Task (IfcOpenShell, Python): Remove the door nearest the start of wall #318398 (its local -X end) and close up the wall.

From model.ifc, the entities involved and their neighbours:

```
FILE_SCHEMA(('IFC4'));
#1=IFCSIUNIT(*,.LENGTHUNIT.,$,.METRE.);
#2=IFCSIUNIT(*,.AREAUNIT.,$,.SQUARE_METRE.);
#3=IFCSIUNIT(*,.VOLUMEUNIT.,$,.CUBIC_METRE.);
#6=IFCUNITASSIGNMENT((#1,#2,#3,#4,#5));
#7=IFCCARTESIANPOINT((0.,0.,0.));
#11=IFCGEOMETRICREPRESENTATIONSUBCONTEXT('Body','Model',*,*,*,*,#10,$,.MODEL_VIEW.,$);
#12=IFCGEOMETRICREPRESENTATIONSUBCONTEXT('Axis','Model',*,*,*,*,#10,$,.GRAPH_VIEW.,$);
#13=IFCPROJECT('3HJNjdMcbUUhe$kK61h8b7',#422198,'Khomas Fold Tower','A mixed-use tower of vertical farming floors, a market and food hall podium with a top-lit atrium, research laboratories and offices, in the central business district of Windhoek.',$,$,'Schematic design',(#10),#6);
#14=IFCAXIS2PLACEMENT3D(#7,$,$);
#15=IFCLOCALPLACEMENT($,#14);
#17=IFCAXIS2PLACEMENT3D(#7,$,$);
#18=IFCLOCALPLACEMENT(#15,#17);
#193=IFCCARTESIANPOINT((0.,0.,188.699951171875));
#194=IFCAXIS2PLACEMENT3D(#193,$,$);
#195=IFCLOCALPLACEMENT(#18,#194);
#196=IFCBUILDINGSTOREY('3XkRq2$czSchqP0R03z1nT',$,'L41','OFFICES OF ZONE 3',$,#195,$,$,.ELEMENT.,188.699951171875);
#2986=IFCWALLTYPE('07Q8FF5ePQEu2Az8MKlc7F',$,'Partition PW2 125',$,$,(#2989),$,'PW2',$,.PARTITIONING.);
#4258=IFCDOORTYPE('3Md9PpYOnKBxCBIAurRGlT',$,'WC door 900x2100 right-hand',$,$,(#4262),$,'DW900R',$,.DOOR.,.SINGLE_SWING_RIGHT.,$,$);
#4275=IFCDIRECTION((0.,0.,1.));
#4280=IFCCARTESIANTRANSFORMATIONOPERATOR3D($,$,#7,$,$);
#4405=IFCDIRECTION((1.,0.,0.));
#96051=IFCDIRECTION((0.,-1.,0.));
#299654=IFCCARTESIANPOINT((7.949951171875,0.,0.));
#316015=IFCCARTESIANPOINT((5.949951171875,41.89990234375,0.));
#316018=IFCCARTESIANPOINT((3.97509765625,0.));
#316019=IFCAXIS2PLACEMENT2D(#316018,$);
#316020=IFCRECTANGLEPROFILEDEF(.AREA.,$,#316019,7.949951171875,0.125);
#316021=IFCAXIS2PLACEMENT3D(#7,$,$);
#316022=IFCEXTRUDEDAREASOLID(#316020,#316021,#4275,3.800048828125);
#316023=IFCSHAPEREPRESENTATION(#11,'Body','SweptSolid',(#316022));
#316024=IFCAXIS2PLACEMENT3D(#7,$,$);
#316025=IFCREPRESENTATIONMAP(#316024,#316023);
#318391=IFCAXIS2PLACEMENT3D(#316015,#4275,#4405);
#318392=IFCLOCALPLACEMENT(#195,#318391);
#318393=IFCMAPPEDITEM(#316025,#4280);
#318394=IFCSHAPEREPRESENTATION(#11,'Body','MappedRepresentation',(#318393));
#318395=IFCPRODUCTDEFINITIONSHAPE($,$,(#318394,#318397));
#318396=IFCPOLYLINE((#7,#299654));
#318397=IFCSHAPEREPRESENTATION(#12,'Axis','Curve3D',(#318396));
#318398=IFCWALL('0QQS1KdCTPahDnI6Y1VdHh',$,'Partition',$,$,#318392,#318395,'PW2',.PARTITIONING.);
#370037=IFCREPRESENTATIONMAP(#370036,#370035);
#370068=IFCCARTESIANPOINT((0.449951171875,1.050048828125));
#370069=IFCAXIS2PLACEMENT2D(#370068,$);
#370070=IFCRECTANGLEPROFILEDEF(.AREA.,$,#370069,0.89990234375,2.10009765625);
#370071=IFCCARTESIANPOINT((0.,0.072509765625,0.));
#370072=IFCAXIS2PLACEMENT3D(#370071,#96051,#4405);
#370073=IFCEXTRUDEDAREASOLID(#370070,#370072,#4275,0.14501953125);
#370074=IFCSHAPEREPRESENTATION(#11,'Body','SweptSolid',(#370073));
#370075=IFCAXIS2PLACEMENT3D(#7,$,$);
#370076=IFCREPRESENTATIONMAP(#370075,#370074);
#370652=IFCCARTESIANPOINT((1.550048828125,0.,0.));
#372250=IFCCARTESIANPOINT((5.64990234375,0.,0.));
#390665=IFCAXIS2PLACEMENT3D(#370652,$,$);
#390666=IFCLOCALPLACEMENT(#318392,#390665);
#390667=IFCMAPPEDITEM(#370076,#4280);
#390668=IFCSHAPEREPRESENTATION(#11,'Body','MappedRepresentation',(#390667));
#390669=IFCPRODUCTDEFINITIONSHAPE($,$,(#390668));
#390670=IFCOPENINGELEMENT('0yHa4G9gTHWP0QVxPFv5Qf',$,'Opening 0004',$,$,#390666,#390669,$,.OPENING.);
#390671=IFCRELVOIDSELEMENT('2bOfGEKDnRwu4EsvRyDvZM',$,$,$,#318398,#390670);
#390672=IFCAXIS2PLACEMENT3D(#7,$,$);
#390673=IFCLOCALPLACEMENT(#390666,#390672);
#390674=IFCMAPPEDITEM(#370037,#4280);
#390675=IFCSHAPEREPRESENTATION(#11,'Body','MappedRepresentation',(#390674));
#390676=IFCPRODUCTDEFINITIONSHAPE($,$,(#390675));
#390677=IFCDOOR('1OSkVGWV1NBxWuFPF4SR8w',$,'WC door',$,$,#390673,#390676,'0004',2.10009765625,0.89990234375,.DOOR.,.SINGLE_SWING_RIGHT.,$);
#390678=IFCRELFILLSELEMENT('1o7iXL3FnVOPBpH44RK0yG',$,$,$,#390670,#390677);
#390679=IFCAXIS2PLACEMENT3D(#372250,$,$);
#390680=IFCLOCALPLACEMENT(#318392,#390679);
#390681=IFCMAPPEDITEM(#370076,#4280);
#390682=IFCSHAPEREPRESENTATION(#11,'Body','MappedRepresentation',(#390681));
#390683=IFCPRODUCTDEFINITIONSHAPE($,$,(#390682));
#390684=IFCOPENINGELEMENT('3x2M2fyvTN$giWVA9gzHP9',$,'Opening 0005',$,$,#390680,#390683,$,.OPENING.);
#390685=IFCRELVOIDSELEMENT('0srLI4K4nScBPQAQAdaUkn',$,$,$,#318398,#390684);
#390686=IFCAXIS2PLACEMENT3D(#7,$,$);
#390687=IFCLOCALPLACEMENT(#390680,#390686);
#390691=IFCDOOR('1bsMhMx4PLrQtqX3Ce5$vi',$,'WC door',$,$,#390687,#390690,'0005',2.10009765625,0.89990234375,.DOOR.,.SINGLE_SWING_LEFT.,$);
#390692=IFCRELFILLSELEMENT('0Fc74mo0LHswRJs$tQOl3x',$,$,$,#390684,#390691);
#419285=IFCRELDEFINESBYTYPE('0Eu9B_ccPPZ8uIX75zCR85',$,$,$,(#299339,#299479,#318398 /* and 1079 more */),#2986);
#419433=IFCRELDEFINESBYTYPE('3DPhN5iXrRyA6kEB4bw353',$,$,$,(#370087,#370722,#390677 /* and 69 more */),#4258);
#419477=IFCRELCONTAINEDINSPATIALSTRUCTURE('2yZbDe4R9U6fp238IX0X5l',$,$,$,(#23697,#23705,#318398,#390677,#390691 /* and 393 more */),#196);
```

```python
import ifcopenshell
import ifcopenshell.api.feature
import ifcopenshell.api.root
import ifcopenshell.geom
import ifcopenshell.util.shape

model = ifcopenshell.open("model.ifc")
settings = ifcopenshell.geom.settings()


def volume(element):
    """Net volume in cubic metres, openings subtracted."""
    shape = ifcopenshell.geom.create_shape(settings, element)
    return ifcopenshell.util.shape.get_volume(shape.geometry)


door = model.by_guid("1OSkVGWV1NBxWuFPF4SR8w")
opening = door.FillsVoids[0].RelatingOpeningElement
wall = opening.VoidsElements[0].RelatingBuildingElement
before = volume(wall)

ifcopenshell.api.root.remove_product(model, product=door)
ifcopenshell.api.feature.remove_feature(model, feature=opening)

after = volume(wall)

print(f"wall volume {before:.3f} -> {after:.3f} m3")

model.write("model-out.ifc")
```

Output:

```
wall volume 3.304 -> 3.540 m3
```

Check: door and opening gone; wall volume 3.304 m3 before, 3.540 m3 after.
